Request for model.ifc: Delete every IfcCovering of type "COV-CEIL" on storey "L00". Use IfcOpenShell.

First a look at what the model holds.

```python
import ifcopenshell
import ifcopenshell.util.element

model = ifcopenshell.open("model.ifc")
print(model.schema)
storey = next(s for s in model.by_type("IfcBuildingStorey") if s.Name == "L00")
coverings = [e for e in ifcopenshell.util.element.get_decomposition(storey) if e.is_a("IfcCovering")]
seen = {}
for e in coverings:
    element_type = ifcopenshell.util.element.get_type(e)
    name = element_type.Name if element_type not in (None, e) else None
    seen[name] = seen.get(name, 0) + 1
for name, count in sorted(seen.items(), key=str):
    print(count, "x", name)
```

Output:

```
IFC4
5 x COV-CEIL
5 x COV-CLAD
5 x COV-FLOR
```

```python
import ifcopenshell
import ifcopenshell.api.root
import ifcopenshell.util.element

model = ifcopenshell.open("model.ifc")

storey = next(s for s in model.by_type("IfcBuildingStorey") if s.Name == "L00")
coverings = [e for e in ifcopenshell.util.element.get_decomposition(storey) if e.is_a("IfcCovering")]
targets = [e for e in coverings if (t := ifcopenshell.util.element.get_type(e)) not in (None, e) and t.Name == "COV-CEIL"]

for e in targets:
    ifcopenshell.api.root.remove_product(model, product=e)
print(len(targets), "removed")

model.write("model_v2.ifc")
```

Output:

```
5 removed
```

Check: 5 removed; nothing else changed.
